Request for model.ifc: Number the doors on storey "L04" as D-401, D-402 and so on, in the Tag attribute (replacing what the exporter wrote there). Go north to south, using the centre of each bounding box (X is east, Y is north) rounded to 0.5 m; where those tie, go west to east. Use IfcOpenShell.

First a look at what the model holds.

```python
import ifcopenshell
import ifcopenshell.util.element
import ifcopenshell.util.placement

model = ifcopenshell.open("model.ifc")
print(model.schema)
storey = next(s for s in model.by_type("IfcBuildingStorey") if s.Name == "L04")
doors = [e for e in ifcopenshell.util.element.get_decomposition(storey) if e.is_a("IfcDoor")]
for e in sorted(doors, key=lambda e: e.id()):
    origin = ifcopenshell.util.placement.get_local_placement(e.ObjectPlacement)[:3, 3]
    print(e.id(), e.Tag, e.Name, origin.round(2) + 0.0, sep=" | ")
```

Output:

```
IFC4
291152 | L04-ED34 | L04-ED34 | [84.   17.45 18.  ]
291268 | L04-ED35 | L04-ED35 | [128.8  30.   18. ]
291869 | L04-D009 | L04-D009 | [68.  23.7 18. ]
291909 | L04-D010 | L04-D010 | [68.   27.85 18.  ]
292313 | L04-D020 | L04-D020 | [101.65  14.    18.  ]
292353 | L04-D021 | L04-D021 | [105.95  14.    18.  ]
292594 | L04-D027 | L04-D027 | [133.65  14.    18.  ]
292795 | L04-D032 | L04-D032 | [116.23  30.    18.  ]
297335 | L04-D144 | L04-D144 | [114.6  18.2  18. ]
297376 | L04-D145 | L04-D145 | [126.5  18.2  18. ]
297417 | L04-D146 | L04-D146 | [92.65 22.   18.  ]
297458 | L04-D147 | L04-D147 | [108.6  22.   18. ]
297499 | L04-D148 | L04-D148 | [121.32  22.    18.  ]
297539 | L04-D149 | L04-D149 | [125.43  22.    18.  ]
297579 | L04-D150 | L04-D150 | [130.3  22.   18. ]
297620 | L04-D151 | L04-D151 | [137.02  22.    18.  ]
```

```python
import ifcopenshell
import ifcopenshell.geom
import ifcopenshell.util.element
import ifcopenshell.util.shape

model = ifcopenshell.open("model.ifc")
settings = ifcopenshell.geom.settings()
settings.set("use-world-coords", True)


def centre(element):
    shape = ifcopenshell.geom.create_shape(settings, element)
    return ifcopenshell.util.shape.get_bbox_centroid(shape.geometry)


storey = next(s for s in model.by_type("IfcBuildingStorey") if s.Name == "L04")
doors = [e for e in ifcopenshell.util.element.get_decomposition(storey) if e.is_a("IfcDoor")]

# Insertion points can sit at a corner or the storey origin, so sort by the geometry (in metres).
centres = {e: centre(e) for e in doors}
doors.sort(key=lambda e: (-round(centres[e][1] / 0.5), centres[e][0]))

for i, e in enumerate(doors, start=1):
    number = f"D-4{i:02d}"
    e.Tag = number
    print(e.id(), number)

model.write("model_updated.ifc")
```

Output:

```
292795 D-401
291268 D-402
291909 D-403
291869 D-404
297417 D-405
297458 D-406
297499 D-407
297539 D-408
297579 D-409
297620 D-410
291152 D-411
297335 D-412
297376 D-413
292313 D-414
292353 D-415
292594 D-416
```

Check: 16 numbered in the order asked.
